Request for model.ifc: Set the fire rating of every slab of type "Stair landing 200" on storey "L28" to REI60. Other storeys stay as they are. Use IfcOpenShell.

First a look at what the model holds.

```python
import ifcopenshell
import ifcopenshell.util.element

model = ifcopenshell.open("model.ifc")
print(model.schema)
storey = next(s for s in model.by_type("IfcBuildingStorey") if s.Name == "L28")
slabs = [e for e in ifcopenshell.util.element.get_decomposition(storey) if e.is_a("IfcSlab")]
seen = {}
for e in slabs:
    element_type = ifcopenshell.util.element.get_type(e)
    key = (element_type.Name if element_type != e and element_type else None, ifcopenshell.util.element.get_pset(e, "Pset_SlabCommon", "FireRating"))
    seen[key] = seen.get(key, 0) + 1
for (name, value), count in sorted(seen.items(), key=str):
    print(count, "x", name, "|", value)
```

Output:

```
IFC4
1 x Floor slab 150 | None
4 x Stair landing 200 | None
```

```python
import ifcopenshell
import ifcopenshell.api.pset
import ifcopenshell.util.element

model = ifcopenshell.open("model.ifc")

storey = next(s for s in model.by_type("IfcBuildingStorey") if s.Name == "L28")
slabs = [e for e in ifcopenshell.util.element.get_decomposition(storey) if e.is_a("IfcSlab")]

count = 0
for e in slabs:
    element_type = ifcopenshell.util.element.get_type(e)
    if element_type in (None, e) or element_type.Name != "Stair landing 200":
        continue
    found = ifcopenshell.util.element.get_pset(e, "Pset_SlabCommon", should_inherit=False)
    if found:
        pset = model.by_id(found["id"])
        if len(ifcopenshell.util.element.get_elements_by_pset(pset)) > 1:
            pset = ifcopenshell.api.pset.unshare_pset(model, products=[e], pset=pset)[0]
    else:
        pset = ifcopenshell.api.pset.add_pset(model, product=e, name="Pset_SlabCommon")
    ifcopenshell.api.pset.edit_pset(model, pset=pset, properties={"FireRating": "REI60"})
    count += 1

print(count, "slabs updated")

model.write("model_rev.ifc")
```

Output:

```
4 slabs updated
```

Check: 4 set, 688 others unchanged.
